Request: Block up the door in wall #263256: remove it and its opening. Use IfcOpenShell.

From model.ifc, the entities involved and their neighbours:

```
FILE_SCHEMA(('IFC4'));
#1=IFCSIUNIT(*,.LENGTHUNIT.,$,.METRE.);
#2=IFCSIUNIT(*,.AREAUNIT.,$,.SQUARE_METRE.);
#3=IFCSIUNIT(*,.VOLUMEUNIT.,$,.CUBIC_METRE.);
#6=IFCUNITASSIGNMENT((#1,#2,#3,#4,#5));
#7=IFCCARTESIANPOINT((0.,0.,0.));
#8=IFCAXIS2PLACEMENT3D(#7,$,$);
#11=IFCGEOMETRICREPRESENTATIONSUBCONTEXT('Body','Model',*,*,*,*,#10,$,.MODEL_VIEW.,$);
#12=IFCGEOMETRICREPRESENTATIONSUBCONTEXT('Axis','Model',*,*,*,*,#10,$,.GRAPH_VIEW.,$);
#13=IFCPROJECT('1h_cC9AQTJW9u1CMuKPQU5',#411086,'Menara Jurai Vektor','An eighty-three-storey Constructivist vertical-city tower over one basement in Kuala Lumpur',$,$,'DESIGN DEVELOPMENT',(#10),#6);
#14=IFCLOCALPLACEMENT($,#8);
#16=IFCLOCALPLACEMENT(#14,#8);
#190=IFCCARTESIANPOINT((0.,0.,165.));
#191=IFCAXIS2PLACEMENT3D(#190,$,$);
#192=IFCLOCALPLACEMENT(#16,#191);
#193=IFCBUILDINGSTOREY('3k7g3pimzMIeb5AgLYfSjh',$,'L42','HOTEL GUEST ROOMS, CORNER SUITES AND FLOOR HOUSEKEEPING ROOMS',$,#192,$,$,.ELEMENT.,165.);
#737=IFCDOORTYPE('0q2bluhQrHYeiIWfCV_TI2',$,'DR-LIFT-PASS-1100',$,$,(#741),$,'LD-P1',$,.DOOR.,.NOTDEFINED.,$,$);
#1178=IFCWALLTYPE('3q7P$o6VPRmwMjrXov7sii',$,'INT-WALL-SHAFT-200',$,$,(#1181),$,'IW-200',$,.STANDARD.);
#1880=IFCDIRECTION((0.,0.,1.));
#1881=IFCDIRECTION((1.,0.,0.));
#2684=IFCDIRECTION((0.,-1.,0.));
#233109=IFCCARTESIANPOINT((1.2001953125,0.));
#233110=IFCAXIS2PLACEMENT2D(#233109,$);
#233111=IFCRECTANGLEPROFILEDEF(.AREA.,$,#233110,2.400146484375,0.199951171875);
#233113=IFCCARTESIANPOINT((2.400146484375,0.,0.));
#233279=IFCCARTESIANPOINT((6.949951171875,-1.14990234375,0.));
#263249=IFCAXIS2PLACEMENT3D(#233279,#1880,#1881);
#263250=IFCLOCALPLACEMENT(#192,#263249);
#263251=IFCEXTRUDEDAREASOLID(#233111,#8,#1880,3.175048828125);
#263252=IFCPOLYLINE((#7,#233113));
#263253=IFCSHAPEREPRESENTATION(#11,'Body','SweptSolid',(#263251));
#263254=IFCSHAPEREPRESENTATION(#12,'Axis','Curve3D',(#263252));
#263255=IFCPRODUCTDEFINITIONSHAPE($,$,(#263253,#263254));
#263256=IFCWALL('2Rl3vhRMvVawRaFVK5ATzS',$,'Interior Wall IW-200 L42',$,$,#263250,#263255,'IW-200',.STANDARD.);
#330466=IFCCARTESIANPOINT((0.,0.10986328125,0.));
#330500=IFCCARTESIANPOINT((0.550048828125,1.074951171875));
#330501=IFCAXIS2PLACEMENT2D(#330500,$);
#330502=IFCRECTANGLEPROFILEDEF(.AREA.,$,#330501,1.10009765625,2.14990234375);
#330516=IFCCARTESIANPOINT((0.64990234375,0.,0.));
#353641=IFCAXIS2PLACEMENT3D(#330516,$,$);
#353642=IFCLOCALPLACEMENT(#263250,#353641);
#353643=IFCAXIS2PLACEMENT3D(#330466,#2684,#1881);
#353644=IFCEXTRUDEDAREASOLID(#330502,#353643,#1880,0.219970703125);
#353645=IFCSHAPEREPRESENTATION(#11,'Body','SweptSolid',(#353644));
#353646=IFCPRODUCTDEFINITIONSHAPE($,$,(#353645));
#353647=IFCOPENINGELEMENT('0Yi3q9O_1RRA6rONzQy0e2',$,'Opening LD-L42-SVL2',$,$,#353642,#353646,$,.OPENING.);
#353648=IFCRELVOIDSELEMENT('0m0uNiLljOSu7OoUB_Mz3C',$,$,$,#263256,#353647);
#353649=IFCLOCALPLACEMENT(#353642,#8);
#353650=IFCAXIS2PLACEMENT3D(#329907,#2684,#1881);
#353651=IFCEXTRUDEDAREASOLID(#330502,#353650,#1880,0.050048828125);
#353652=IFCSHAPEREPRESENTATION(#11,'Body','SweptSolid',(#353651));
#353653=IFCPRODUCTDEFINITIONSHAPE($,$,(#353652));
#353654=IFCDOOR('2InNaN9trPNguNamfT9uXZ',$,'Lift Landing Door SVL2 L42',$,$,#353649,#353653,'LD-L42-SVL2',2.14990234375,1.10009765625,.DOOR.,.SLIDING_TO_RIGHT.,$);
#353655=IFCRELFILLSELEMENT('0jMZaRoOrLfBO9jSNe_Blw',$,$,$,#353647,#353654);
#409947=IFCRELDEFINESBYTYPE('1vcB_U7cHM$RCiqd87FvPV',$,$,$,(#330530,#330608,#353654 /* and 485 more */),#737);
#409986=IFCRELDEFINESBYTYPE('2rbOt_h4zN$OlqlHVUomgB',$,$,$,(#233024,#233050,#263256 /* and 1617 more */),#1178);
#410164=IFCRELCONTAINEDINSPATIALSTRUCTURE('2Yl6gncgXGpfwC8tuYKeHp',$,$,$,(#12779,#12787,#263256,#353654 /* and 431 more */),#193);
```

```python
import ifcopenshell
import ifcopenshell.api.feature
import ifcopenshell.api.root
import ifcopenshell.geom
import ifcopenshell.util.shape

model = ifcopenshell.open("model.ifc")
settings = ifcopenshell.geom.settings()


def volume(element):
    """Net volume in cubic metres, openings subtracted."""
    shape = ifcopenshell.geom.create_shape(settings, element)
    return ifcopenshell.util.shape.get_volume(shape.geometry)


door = model.by_id(353654)
opening = door.FillsVoids[0].RelatingOpeningElement
wall = opening.VoidsElements[0].RelatingBuildingElement
before = volume(wall)

ifcopenshell.api.root.remove_product(model, product=door)
ifcopenshell.api.feature.remove_feature(model, feature=opening)

after = volume(wall)

print(f"wall volume {before:.3f} -> {after:.3f} m3")

model.write("model_v2.ifc")
```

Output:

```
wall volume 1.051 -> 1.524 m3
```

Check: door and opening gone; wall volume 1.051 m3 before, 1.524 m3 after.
